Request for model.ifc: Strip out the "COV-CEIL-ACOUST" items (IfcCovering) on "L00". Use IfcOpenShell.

First a look at what the model holds.

```python
import ifcopenshell
import ifcopenshell.util.element

model = ifcopenshell.open("model.ifc")
print(model.schema)
storey = next(s for s in model.by_type("IfcBuildingStorey") if s.Name == "L00")
coverings = [e for e in ifcopenshell.util.element.get_decomposition(storey) if e.is_a("IfcCovering")]
seen = {}
for e in coverings:
    element_type = ifcopenshell.util.element.get_type(e)
    name = element_type.Name if element_type not in (None, e) else None
    seen[name] = seen.get(name, 0) + 1
for name, count in sorted(seen.items(), key=str):
    print(count, "x", name)
```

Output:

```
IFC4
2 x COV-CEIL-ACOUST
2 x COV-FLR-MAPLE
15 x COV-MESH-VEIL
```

```python
import ifcopenshell
import ifcopenshell.api.root
import ifcopenshell.util.element

model = ifcopenshell.open("model.ifc")

storey = next(s for s in model.by_type("IfcBuildingStorey") if s.Name == "L00")
coverings = [e for e in ifcopenshell.util.element.get_decomposition(storey) if e.is_a("IfcCovering")]
targets = [e for e in coverings if (t := ifcopenshell.util.element.get_type(e)) not in (None, e) and t.Name == "COV-CEIL-ACOUST"]

for e in targets:
    ifcopenshell.api.root.remove_product(model, product=e)
print(len(targets), "removed")

model.write("model_edited.ifc")
```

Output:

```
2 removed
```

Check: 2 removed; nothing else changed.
